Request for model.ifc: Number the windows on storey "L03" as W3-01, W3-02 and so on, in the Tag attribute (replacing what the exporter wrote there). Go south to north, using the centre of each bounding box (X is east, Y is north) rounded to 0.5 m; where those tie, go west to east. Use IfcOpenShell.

First a look at what the model holds.

```python
import ifcopenshell
import ifcopenshell.util.element
import ifcopenshell.util.placement

model = ifcopenshell.open("model.ifc")
print(model.schema)
storey = next(s for s in model.by_type("IfcBuildingStorey") if s.Name == "L03")
windows = [e for e in ifcopenshell.util.element.get_decomposition(storey) if e.is_a("IfcWindow")]
for e in sorted(windows, key=lambda e: e.id()):
    origin = ifcopenshell.util.placement.get_local_placement(e.ObjectPlacement)[:3, 3]
    print(e.id(), e.Tag, e.Name, origin.round(2) + 0.0, sep=" | ")
```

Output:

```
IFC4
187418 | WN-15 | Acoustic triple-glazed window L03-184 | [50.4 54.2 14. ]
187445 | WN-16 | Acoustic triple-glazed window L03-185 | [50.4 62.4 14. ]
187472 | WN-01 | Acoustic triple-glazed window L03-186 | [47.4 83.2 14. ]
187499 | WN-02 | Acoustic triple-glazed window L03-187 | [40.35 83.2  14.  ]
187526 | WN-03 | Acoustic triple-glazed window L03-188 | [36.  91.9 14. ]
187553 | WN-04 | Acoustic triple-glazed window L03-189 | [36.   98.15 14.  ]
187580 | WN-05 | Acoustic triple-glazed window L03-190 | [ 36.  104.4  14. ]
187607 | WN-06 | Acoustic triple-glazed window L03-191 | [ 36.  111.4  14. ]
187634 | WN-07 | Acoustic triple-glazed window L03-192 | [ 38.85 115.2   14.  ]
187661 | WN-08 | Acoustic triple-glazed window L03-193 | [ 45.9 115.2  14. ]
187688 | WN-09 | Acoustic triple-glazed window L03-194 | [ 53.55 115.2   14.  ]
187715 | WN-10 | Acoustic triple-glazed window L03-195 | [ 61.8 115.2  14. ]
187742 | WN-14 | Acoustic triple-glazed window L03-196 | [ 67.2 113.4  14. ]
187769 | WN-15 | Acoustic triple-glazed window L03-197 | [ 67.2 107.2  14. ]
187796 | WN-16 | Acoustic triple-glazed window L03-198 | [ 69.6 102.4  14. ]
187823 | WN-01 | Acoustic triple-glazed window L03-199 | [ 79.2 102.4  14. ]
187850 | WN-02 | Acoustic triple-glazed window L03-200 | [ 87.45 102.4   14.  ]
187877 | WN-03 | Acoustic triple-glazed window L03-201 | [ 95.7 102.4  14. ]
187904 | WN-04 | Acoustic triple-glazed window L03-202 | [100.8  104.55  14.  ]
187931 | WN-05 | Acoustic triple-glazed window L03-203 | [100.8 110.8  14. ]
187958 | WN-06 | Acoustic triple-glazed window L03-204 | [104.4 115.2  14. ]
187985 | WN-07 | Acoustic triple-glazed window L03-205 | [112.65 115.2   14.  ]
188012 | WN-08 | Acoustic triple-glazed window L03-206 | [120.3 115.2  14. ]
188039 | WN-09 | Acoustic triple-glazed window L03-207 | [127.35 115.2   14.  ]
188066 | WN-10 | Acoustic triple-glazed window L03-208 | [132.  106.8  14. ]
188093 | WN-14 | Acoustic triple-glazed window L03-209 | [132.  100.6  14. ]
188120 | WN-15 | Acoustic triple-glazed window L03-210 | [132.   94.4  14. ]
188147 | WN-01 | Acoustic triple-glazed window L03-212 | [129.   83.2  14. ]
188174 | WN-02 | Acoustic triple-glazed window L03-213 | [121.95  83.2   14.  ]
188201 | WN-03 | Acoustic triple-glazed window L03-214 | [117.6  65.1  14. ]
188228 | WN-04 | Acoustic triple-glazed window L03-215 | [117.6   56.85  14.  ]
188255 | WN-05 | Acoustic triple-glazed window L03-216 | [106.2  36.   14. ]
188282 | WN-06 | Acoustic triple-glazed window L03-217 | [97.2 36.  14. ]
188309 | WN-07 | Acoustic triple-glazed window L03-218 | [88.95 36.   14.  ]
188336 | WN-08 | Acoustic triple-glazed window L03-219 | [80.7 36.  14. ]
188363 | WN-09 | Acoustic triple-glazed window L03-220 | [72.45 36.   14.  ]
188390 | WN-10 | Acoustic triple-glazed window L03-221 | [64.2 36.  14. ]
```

```python
import ifcopenshell
import ifcopenshell.geom
import ifcopenshell.util.element
import ifcopenshell.util.shape

model = ifcopenshell.open("model.ifc")
settings = ifcopenshell.geom.settings()
settings.set("use-world-coords", True)


def centre(element):
    shape = ifcopenshell.geom.create_shape(settings, element)
    return ifcopenshell.util.shape.get_bbox_centroid(shape.geometry)


storey = next(s for s in model.by_type("IfcBuildingStorey") if s.Name == "L03")
windows = [e for e in ifcopenshell.util.element.get_decomposition(storey) if e.is_a("IfcWindow")]

# Insertion points can sit at a corner or the storey origin, so sort by the geometry (in metres).
centres = {e: centre(e) for e in windows}
windows.sort(key=lambda e: (round(centres[e][1] / 0.5), centres[e][0]))

for i, e in enumerate(windows, start=1):
    number = f"W3-{i:02d}"
    e.Tag = number
    print(e.id(), number)

model.write("model_rev.ifc")
```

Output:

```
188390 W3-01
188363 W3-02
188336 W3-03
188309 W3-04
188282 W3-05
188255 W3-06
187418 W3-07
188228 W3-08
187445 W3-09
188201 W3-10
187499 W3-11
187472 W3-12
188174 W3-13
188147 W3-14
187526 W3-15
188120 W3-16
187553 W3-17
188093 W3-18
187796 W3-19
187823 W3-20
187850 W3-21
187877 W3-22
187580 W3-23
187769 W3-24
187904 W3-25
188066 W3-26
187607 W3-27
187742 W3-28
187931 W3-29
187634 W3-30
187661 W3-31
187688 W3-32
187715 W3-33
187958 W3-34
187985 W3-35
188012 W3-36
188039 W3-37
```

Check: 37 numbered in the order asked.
